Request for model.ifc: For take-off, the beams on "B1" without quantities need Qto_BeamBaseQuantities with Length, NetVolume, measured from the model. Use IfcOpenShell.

First a look at what the model holds.

```python
import ifcopenshell
import ifcopenshell.util.element
import ifcopenshell.util.unit

model = ifcopenshell.open("model.ifc")
print(model.schema)
for unit_type in ("LENGTHUNIT", "AREAUNIT", "VOLUMEUNIT"):
    print(unit_type, ifcopenshell.util.unit.calculate_unit_scale(model, unit_type))
storey = next(s for s in model.by_type("IfcBuildingStorey") if s.Name == "B1")
beams = [e for e in ifcopenshell.util.element.get_decomposition(storey) if e.is_a("IfcBeam")]
for e in sorted(beams, key=lambda e: e.id()):
    print(e.id(), e.is_a(), e.Name, list(ifcopenshell.util.element.get_psets(e, qtos_only=True)), sep=" | ")
```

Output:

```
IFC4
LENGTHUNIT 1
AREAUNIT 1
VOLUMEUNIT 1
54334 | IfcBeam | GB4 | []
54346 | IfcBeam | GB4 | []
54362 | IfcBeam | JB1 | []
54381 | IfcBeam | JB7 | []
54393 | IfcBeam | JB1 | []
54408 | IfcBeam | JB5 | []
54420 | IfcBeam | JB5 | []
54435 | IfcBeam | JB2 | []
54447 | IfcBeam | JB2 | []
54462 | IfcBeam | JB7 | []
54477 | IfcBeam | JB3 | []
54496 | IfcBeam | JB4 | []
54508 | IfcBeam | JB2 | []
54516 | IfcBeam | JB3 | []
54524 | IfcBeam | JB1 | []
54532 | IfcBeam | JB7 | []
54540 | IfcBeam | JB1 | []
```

```python
import ifcopenshell
import ifcopenshell.api.pset
import ifcopenshell.geom
import ifcopenshell.util.element
import ifcopenshell.util.shape
import ifcopenshell.util.unit

model = ifcopenshell.open("model.ifc")
unit_scale = ifcopenshell.util.unit.calculate_unit_scale(model)
volume_scale = ifcopenshell.util.unit.calculate_unit_scale(model, "VOLUMEUNIT")
settings = ifcopenshell.geom.settings()

storey = next(s for s in model.by_type("IfcBuildingStorey") if s.Name == "B1")
beams = [e for e in ifcopenshell.util.element.get_decomposition(storey) if e.is_a("IfcBeam")]

for e in sorted(beams, key=lambda e: e.id()):
    if ifcopenshell.util.element.get_psets(e, qtos_only=True, should_inherit=False):
        continue
    # Geometry comes back in metres, in the element's own axes.
    shape = ifcopenshell.geom.create_shape(settings, e)
    values = {
        "Length": ifcopenshell.util.shape.get_max_xyz(shape.geometry) / unit_scale,
        "NetVolume": ifcopenshell.util.shape.get_volume(shape.geometry) / volume_scale,
    }
    qto = ifcopenshell.api.pset.add_qto(model, product=e, name="Qto_BeamBaseQuantities")
    ifcopenshell.api.pset.edit_qto(model, qto=qto, properties=values)
    print(e.id(), {k: round(v, 3) for k, v in values.items()})

model.write("model_rev.ifc")
```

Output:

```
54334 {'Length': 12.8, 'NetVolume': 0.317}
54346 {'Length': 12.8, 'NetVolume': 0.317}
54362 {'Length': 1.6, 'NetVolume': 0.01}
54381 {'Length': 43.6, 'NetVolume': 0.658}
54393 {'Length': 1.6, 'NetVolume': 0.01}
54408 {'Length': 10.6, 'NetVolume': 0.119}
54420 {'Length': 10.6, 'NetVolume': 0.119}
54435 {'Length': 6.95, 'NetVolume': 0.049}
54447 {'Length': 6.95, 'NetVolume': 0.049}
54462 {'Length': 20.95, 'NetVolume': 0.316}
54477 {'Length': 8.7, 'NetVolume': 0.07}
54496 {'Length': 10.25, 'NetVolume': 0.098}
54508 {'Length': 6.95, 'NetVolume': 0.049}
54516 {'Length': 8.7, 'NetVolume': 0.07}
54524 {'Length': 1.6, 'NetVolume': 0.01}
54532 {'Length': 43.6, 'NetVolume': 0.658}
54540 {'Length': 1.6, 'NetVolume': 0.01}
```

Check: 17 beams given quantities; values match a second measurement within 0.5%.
